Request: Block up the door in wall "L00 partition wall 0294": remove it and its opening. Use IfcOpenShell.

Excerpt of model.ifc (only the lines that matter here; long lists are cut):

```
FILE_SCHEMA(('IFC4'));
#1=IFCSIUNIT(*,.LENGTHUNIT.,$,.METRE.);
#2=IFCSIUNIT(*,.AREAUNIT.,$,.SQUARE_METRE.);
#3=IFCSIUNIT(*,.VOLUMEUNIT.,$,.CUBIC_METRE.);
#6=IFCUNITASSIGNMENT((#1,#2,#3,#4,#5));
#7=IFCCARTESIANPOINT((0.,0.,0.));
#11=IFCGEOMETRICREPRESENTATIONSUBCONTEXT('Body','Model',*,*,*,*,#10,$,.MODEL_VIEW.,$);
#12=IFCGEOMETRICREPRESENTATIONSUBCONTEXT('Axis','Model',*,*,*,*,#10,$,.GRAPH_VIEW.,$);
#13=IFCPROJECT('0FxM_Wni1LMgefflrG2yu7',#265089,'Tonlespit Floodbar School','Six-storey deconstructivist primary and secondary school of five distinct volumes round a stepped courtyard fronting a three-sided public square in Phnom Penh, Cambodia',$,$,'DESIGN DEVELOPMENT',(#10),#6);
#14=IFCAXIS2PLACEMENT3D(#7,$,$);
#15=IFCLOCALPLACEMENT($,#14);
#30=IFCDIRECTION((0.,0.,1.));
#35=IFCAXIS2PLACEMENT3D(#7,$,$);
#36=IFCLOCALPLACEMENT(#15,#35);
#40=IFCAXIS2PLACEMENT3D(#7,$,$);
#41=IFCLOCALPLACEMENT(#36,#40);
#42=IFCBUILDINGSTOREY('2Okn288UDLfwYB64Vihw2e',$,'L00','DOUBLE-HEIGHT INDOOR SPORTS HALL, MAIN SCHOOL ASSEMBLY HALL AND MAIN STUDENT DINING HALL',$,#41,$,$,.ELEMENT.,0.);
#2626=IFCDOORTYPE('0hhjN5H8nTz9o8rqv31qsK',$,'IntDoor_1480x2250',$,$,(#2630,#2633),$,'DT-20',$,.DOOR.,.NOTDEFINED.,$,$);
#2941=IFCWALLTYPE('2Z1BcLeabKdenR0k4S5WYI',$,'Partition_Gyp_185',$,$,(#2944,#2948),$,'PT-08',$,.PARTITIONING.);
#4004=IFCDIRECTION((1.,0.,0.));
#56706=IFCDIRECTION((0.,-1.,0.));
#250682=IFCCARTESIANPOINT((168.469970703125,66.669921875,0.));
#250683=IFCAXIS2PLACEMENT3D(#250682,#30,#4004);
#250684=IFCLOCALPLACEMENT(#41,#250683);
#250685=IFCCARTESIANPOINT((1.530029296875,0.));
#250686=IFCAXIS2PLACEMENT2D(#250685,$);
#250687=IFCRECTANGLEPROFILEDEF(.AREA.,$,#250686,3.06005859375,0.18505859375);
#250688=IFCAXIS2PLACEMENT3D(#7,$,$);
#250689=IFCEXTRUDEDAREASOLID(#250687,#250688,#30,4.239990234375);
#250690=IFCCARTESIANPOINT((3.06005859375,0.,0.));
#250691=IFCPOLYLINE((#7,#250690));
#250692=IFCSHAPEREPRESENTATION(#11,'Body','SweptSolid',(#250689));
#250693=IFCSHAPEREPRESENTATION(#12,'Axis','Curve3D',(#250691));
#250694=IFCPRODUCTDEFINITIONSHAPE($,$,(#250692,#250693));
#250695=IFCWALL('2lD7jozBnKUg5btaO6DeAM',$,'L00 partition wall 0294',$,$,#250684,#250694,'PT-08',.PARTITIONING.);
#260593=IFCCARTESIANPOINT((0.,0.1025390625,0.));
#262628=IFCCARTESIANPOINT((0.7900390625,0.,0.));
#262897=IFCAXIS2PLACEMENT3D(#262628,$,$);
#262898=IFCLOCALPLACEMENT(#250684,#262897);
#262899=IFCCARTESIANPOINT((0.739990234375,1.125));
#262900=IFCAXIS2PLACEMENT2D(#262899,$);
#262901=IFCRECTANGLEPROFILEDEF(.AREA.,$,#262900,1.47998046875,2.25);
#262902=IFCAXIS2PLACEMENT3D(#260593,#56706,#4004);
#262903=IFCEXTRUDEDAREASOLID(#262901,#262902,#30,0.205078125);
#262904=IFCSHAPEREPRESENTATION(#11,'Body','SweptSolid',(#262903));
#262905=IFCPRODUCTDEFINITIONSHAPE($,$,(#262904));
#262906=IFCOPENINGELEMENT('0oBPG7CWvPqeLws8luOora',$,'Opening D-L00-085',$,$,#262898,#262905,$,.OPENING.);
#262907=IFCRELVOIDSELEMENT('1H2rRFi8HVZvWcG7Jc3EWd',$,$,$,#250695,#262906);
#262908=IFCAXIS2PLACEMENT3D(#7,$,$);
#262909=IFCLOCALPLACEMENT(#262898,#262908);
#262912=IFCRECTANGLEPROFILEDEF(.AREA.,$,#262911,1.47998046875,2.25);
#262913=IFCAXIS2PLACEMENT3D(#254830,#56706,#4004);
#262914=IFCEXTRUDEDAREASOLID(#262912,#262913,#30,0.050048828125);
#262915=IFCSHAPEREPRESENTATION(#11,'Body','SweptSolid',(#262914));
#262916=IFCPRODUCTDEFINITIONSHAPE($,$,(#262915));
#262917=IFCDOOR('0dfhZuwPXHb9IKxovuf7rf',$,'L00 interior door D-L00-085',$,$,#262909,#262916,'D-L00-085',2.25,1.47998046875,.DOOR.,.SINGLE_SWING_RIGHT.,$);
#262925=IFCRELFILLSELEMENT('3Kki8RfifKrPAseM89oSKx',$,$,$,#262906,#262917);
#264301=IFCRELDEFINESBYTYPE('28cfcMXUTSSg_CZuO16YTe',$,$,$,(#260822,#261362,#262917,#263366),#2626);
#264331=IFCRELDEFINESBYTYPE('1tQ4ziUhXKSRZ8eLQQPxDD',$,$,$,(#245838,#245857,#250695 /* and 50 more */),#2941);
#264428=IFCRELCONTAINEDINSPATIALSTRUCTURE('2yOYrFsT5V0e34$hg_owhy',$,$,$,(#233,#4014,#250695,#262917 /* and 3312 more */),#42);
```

```python
import ifcopenshell
import ifcopenshell.api.feature
import ifcopenshell.api.root
import ifcopenshell.geom
import ifcopenshell.util.shape

model = ifcopenshell.open("model.ifc")
settings = ifcopenshell.geom.settings()


def volume(element):
    """Net volume in cubic metres, openings subtracted."""
    shape = ifcopenshell.geom.create_shape(settings, element)
    return ifcopenshell.util.shape.get_volume(shape.geometry)


door = model.by_guid("0dfhZuwPXHb9IKxovuf7rf")
opening = door.FillsVoids[0].RelatingOpeningElement
wall = opening.VoidsElements[0].RelatingBuildingElement
before = volume(wall)

ifcopenshell.api.root.remove_product(model, product=door)
ifcopenshell.api.feature.remove_feature(model, feature=opening)

after = volume(wall)

print(f"wall volume {before:.3f} -> {after:.3f} m3")

model.write("model_updated.ifc")
```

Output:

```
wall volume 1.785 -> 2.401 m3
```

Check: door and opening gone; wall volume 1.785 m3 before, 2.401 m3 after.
